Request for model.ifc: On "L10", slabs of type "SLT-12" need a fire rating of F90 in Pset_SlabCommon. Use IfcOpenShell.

First a look at what the model holds.

```python
import ifcopenshell
import ifcopenshell.util.element

model = ifcopenshell.open("model.ifc")
print(model.schema)
storey = next(s for s in model.by_type("IfcBuildingStorey") if s.Name == "L10")
slabs = [e for e in ifcopenshell.util.element.get_decomposition(storey) if e.is_a("IfcSlab")]
seen = {}
for e in slabs:
    element_type = ifcopenshell.util.element.get_type(e)
    key = (element_type.Name if element_type != e and element_type else None, ifcopenshell.util.element.get_pset(e, "Pset_SlabCommon", "FireRating"))
    seen[key] = seen.get(key, 0) + 1
for (name, value), count in sorted(seen.items(), key=str):
    print(count, "x", name, "|", value)
```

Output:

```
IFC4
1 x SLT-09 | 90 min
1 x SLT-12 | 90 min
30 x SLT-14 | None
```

```python
import ifcopenshell
import ifcopenshell.api.pset
import ifcopenshell.util.element

model = ifcopenshell.open("model.ifc")

storey = next(s for s in model.by_type("IfcBuildingStorey") if s.Name == "L10")
slabs = [e for e in ifcopenshell.util.element.get_decomposition(storey) if e.is_a("IfcSlab")]

count = 0
for e in slabs:
    element_type = ifcopenshell.util.element.get_type(e)
    if element_type in (None, e) or element_type.Name != "SLT-12":
        continue
    # add_pset returns the element's existing set when there is one.
    pset = ifcopenshell.api.pset.add_pset(model, product=e, name="Pset_SlabCommon")
    ifcopenshell.api.pset.edit_pset(model, pset=pset, properties={"FireRating": "F90"})
    count += 1

print(count, "slabs updated")

model.write("model_rev.ifc")
```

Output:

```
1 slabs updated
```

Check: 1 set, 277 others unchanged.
